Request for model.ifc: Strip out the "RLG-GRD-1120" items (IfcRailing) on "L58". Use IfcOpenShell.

First a look at what the model holds.

```python
import ifcopenshell
import ifcopenshell.util.element

model = ifcopenshell.open("model.ifc")
print(model.schema)
storey = next(s for s in model.by_type("IfcBuildingStorey") if s.Name == "L58")
railings = [e for e in ifcopenshell.util.element.get_decomposition(storey) if e.is_a("IfcRailing")]
seen = {}
for e in railings:
    element_type = ifcopenshell.util.element.get_type(e)
    name = element_type.Name if element_type not in (None, e) else None
    seen[name] = seen.get(name, 0) + 1
for name, count in sorted(seen.items(), key=str):
    print(count, "x", name)
```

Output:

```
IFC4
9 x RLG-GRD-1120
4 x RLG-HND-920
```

```python
import ifcopenshell
import ifcopenshell.api.root
import ifcopenshell.util.element

model = ifcopenshell.open("model.ifc")

storey = next(s for s in model.by_type("IfcBuildingStorey") if s.Name == "L58")
railings = [e for e in ifcopenshell.util.element.get_decomposition(storey) if e.is_a("IfcRailing")]
targets = [e for e in railings if (t := ifcopenshell.util.element.get_type(e)) not in (None, e) and t.Name == "RLG-GRD-1120"]

for e in targets:
    ifcopenshell.api.root.remove_product(model, product=e)
print(len(targets), "removed")

model.write("model_rev.ifc")
```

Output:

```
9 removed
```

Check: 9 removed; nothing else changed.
